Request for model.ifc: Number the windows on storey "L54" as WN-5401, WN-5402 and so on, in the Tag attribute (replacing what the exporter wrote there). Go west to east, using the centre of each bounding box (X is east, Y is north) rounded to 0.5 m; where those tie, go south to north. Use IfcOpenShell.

First a look at what the model holds.

```python
import ifcopenshell
import ifcopenshell.util.element
import ifcopenshell.util.placement

model = ifcopenshell.open("model.ifc")
print(model.schema)
storey = next(s for s in model.by_type("IfcBuildingStorey") if s.Name == "L54")
windows = [e for e in ifcopenshell.util.element.get_decomposition(storey) if e.is_a("IfcWindow")]
for e in sorted(windows, key=lambda e: e.id()):
    origin = ifcopenshell.util.placement.get_local_placement(e.ObjectPlacement)[:3, 3]
    print(e.id(), e.Tag, e.Name, origin.round(2) + 0.0, sep=" | ")
```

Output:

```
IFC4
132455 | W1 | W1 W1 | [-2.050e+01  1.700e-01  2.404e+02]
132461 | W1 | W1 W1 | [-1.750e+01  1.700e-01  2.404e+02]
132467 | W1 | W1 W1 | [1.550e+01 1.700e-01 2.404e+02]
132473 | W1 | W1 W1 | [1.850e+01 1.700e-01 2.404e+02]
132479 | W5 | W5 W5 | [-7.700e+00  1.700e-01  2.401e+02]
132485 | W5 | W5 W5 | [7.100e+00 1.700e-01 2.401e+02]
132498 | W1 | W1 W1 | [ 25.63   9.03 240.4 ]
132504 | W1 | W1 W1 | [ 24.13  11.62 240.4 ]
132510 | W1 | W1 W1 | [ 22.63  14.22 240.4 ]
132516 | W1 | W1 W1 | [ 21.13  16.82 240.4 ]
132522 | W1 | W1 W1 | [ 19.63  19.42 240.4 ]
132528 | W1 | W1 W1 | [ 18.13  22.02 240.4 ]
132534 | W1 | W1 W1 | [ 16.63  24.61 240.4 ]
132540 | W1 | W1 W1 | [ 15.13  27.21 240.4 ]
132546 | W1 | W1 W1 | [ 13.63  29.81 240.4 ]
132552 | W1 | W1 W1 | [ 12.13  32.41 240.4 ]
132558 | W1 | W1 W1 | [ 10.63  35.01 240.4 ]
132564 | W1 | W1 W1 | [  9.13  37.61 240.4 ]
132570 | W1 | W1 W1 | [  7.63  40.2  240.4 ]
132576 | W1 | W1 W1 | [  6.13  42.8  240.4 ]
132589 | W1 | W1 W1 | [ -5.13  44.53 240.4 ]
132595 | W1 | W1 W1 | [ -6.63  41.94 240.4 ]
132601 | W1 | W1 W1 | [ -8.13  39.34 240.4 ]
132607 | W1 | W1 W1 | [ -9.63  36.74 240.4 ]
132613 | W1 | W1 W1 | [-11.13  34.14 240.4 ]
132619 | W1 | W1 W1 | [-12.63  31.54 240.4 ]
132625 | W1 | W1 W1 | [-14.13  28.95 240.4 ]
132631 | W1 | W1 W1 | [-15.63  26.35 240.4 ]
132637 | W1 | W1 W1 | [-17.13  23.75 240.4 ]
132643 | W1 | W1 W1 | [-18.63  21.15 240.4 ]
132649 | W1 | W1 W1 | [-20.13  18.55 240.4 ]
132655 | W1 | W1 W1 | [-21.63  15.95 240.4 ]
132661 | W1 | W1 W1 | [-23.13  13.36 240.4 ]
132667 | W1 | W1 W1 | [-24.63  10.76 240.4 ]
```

```python
import ifcopenshell
import ifcopenshell.geom
import ifcopenshell.util.element
import ifcopenshell.util.shape

model = ifcopenshell.open("model.ifc")
settings = ifcopenshell.geom.settings()
settings.set("use-world-coords", True)


def centre(element):
    shape = ifcopenshell.geom.create_shape(settings, element)
    return ifcopenshell.util.shape.get_bbox_centroid(shape.geometry)


storey = next(s for s in model.by_type("IfcBuildingStorey") if s.Name == "L54")
windows = [e for e in ifcopenshell.util.element.get_decomposition(storey) if e.is_a("IfcWindow")]

# Insertion points can sit at a corner or the storey origin, so sort by the geometry (in metres).
centres = {e: centre(e) for e in windows}
windows.sort(key=lambda e: (round(centres[e][0] / 0.5), centres[e][1]))

for i, e in enumerate(windows, start=1):
    number = f"WN-54{i:02d}"
    e.Tag = number
    print(e.id(), number)

model.write("model_rev.ifc")
```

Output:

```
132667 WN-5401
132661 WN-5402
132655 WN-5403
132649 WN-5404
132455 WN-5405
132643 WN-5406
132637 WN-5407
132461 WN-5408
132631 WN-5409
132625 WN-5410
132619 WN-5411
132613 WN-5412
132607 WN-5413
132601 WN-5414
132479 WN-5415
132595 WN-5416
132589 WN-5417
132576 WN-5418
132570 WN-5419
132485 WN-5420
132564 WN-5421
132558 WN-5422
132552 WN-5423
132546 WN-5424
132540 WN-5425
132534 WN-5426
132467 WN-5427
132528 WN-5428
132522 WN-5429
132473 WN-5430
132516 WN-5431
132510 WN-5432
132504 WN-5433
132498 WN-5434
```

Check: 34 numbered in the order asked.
